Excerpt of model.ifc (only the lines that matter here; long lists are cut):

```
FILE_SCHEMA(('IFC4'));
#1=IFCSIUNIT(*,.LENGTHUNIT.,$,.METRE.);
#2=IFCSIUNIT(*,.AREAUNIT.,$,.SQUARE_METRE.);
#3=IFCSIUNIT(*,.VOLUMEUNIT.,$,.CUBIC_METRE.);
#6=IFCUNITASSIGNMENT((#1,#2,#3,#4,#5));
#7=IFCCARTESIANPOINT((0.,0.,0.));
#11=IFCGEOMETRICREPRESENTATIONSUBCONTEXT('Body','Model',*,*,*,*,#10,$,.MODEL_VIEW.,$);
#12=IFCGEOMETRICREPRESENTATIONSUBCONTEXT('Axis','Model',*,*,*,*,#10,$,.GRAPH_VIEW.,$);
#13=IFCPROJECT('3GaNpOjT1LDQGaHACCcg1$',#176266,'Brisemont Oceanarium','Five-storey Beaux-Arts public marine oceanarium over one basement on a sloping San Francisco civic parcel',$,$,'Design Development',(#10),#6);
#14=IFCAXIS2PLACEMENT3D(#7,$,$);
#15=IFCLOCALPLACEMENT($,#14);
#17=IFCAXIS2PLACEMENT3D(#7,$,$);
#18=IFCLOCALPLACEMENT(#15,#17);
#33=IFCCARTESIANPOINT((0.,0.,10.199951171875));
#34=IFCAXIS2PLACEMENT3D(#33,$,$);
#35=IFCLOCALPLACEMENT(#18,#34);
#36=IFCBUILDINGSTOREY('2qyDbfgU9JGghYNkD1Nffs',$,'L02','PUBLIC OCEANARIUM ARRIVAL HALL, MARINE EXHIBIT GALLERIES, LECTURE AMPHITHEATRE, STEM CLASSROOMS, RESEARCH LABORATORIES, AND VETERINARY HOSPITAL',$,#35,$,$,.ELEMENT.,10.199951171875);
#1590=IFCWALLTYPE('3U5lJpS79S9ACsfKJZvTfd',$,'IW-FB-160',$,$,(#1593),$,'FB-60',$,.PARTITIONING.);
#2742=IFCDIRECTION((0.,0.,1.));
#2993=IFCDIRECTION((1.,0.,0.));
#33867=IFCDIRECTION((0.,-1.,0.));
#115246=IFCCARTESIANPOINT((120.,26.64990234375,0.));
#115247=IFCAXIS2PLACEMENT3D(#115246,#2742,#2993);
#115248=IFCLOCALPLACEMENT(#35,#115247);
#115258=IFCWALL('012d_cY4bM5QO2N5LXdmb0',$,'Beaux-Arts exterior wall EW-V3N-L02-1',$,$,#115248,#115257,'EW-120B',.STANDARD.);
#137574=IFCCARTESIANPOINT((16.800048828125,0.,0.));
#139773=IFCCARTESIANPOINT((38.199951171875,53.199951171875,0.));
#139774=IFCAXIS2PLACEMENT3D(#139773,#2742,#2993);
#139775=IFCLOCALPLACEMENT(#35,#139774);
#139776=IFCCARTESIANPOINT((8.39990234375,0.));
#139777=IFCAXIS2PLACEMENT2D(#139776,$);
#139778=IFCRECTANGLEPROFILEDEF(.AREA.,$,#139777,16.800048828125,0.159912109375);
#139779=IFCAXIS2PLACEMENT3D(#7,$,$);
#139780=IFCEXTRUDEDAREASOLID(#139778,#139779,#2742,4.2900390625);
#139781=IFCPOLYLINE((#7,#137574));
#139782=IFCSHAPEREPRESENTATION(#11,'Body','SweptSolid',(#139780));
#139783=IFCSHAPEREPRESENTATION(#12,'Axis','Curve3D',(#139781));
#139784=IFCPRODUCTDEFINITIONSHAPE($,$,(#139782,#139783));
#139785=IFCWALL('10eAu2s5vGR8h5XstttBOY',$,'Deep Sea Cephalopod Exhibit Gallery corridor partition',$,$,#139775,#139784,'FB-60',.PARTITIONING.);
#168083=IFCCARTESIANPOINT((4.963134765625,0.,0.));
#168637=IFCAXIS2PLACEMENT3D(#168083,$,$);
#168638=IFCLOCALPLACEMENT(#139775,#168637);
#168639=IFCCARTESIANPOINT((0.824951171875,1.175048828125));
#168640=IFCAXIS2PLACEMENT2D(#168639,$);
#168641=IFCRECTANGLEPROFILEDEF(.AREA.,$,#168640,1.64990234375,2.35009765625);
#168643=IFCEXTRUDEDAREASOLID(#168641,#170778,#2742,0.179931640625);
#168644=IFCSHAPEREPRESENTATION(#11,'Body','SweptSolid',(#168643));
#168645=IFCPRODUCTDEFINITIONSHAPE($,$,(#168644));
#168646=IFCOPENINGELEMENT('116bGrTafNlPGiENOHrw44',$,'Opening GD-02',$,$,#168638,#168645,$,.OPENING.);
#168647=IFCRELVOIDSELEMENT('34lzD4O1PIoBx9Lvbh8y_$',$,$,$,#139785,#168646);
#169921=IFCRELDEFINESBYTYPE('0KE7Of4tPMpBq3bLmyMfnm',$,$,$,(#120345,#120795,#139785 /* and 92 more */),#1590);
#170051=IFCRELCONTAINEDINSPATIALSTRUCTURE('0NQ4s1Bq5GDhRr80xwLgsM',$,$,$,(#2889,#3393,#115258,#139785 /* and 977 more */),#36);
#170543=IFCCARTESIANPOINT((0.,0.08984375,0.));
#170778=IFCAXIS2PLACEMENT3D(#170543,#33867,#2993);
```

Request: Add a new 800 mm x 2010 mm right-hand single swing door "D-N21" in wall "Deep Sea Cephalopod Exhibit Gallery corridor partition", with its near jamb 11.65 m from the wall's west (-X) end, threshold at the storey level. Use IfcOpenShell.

```python
import numpy as np
import ifcopenshell
import ifcopenshell.api.feature
import ifcopenshell.api.geometry
import ifcopenshell.api.root
import ifcopenshell.api.spatial
import ifcopenshell.geom
import ifcopenshell.util.element
import ifcopenshell.util.placement
import ifcopenshell.util.representation
import ifcopenshell.util.shape
import ifcopenshell.util.unit

model = ifcopenshell.open("model.ifc")
unit_scale = ifcopenshell.util.unit.calculate_unit_scale(model)
settings = ifcopenshell.geom.settings()


def volume(element):
    """Net volume in cubic metres, openings subtracted."""
    shape = ifcopenshell.geom.create_shape(settings, element)
    return ifcopenshell.util.shape.get_volume(shape.geometry)


wall = model.by_guid("10eAu2s5vGR8h5XstttBOY")
storey = ifcopenshell.util.element.get_container(wall, ifc_class="IfcBuildingStorey")
context = ifcopenshell.util.representation.get_context(model, "Model", "Body", "MODEL_VIEW")
before = volume(wall)

width, height, from_end, sill = 0.8, 2.01, 11.65, 0.0  # metres

# The wall runs along its own X axis, and the end named is its -X end.
wall_shape = ifcopenshell.geom.create_shape(settings, wall)
x, y, z = ifcopenshell.util.shape.get_vertices(wall_shape.geometry).T
start = x.min() + from_end
face, thickness = float(y.min()), float(y.max() - y.min())
wall_matrix = ifcopenshell.util.placement.get_local_placement(wall.ObjectPlacement)
level = ifcopenshell.util.placement.get_local_placement(storey.ObjectPlacement)[2, 3]


def in_wall(x, y):
    """Placement at x, y metres in the wall's axes, at sill height."""
    matrix = wall_matrix.copy()
    matrix[:, 3] = wall_matrix @ np.array([x / unit_scale, y / unit_scale, 0.0, 1.0])
    matrix[2, 3] = level + sill / unit_scale
    return matrix


# Opening: a box that overshoots both wall faces by 50 mm.
opening = ifcopenshell.api.root.create_entity(model, ifc_class="IfcOpeningElement", predefined_type="OPENING")
box = ifcopenshell.api.geometry.add_wall_representation(
    model, context=context, length=width, height=height, thickness=thickness + 0.1
)
ifcopenshell.api.geometry.assign_representation(model, product=opening, representation=box)
ifcopenshell.api.geometry.edit_object_placement(model, product=opening, matrix=in_wall(start, face - 0.05), is_si=False)
ifcopenshell.api.feature.add_feature(model, feature=opening, element=wall)

door = ifcopenshell.api.root.create_entity(model, ifc_class="IfcDoor", name="D-N21", predefined_type="DOOR")
door.OverallWidth, door.OverallHeight = width / unit_scale, height / unit_scale
door.OperationType = "SINGLE_SWING_RIGHT"
body = ifcopenshell.api.geometry.add_door_representation(
    model,
    context=context,
    overall_width=door.OverallWidth,
    overall_height=door.OverallHeight,
    operation_type="SINGLE_SWING_RIGHT",
    lining_properties={"LiningDepth": thickness / unit_scale, "ThresholdDepth": thickness / unit_scale},
)
ifcopenshell.api.geometry.assign_representation(model, product=door, representation=body)
ifcopenshell.api.spatial.assign_container(model, products=[door], relating_structure=storey)
ifcopenshell.api.feature.add_filling(model, opening=opening, element=door)

# The lining spans the wall, so the door starts at the wall face.
ifcopenshell.api.geometry.edit_object_placement(model, product=door, matrix=in_wall(start, face), is_si=False)

after = volume(wall)

print(f"wall volume {before:.3f} -> {after:.3f} m3")

model.write("model_updated.ifc")
```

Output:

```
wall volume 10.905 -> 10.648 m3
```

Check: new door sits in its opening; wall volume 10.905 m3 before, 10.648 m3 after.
